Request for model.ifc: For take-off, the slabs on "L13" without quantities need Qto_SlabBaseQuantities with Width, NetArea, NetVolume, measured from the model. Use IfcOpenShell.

First a look at what the model holds.

```python
import ifcopenshell
import ifcopenshell.util.element
import ifcopenshell.util.unit

model = ifcopenshell.open("model.ifc")
print(model.schema)
for unit_type in ("LENGTHUNIT", "AREAUNIT", "VOLUMEUNIT"):
    print(unit_type, ifcopenshell.util.unit.calculate_unit_scale(model, unit_type))
storey = next(s for s in model.by_type("IfcBuildingStorey") if s.Name == "L13")
slabs = [e for e in ifcopenshell.util.element.get_decomposition(storey) if e.is_a("IfcSlab")]
for e in sorted(slabs, key=lambda e: e.id()):
    print(e.id(), e.is_a(), e.Name, list(ifcopenshell.util.element.get_psets(e, qtos_only=True)), sep=" | ")
```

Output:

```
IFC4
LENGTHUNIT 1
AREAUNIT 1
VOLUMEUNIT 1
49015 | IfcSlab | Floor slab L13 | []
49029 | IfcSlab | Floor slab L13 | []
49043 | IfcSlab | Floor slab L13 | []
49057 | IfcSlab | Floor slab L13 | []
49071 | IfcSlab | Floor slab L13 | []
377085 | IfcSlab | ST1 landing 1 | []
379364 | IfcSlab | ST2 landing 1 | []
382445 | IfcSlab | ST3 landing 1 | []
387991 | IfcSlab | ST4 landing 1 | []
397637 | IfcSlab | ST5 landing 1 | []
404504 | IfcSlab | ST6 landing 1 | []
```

```python
import ifcopenshell
import ifcopenshell.api.pset
import ifcopenshell.geom
import ifcopenshell.util.element
import ifcopenshell.util.shape
import ifcopenshell.util.unit

model = ifcopenshell.open("model.ifc")
unit_scale = ifcopenshell.util.unit.calculate_unit_scale(model)
area_scale = ifcopenshell.util.unit.calculate_unit_scale(model, "AREAUNIT")
volume_scale = ifcopenshell.util.unit.calculate_unit_scale(model, "VOLUMEUNIT")
settings = ifcopenshell.geom.settings()

storey = next(s for s in model.by_type("IfcBuildingStorey") if s.Name == "L13")
slabs = [e for e in ifcopenshell.util.element.get_decomposition(storey) if e.is_a("IfcSlab")]

for e in sorted(slabs, key=lambda e: e.id()):
    if ifcopenshell.util.element.get_psets(e, qtos_only=True, should_inherit=False):
        continue
    # Geometry comes back in metres, in the element's own axes.
    shape = ifcopenshell.geom.create_shape(settings, e)
    values = {
        "Width": ifcopenshell.util.shape.get_z(shape.geometry) / unit_scale,
        "NetArea": ifcopenshell.util.shape.get_footprint_area(shape.geometry) / area_scale,
        "NetVolume": ifcopenshell.util.shape.get_volume(shape.geometry) / volume_scale,
    }
    qto = ifcopenshell.api.pset.add_qto(model, product=e, name="Qto_SlabBaseQuantities")
    ifcopenshell.api.pset.edit_qto(model, qto=qto, properties=values)
    print(e.id(), {k: round(v, 3) for k, v in values.items()})

model.write("model-out.ifc")
```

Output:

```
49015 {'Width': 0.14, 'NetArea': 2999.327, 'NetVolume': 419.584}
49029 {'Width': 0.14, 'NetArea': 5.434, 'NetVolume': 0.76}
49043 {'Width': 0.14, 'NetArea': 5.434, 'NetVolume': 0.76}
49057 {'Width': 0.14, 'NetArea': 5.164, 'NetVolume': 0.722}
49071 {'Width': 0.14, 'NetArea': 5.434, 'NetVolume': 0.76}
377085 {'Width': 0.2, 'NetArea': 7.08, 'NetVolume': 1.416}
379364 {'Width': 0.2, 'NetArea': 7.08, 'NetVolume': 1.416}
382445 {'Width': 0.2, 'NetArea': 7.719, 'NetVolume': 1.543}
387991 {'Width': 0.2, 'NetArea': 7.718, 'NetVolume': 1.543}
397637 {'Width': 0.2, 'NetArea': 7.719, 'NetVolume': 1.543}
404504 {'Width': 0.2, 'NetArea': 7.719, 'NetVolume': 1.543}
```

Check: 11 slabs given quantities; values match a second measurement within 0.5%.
